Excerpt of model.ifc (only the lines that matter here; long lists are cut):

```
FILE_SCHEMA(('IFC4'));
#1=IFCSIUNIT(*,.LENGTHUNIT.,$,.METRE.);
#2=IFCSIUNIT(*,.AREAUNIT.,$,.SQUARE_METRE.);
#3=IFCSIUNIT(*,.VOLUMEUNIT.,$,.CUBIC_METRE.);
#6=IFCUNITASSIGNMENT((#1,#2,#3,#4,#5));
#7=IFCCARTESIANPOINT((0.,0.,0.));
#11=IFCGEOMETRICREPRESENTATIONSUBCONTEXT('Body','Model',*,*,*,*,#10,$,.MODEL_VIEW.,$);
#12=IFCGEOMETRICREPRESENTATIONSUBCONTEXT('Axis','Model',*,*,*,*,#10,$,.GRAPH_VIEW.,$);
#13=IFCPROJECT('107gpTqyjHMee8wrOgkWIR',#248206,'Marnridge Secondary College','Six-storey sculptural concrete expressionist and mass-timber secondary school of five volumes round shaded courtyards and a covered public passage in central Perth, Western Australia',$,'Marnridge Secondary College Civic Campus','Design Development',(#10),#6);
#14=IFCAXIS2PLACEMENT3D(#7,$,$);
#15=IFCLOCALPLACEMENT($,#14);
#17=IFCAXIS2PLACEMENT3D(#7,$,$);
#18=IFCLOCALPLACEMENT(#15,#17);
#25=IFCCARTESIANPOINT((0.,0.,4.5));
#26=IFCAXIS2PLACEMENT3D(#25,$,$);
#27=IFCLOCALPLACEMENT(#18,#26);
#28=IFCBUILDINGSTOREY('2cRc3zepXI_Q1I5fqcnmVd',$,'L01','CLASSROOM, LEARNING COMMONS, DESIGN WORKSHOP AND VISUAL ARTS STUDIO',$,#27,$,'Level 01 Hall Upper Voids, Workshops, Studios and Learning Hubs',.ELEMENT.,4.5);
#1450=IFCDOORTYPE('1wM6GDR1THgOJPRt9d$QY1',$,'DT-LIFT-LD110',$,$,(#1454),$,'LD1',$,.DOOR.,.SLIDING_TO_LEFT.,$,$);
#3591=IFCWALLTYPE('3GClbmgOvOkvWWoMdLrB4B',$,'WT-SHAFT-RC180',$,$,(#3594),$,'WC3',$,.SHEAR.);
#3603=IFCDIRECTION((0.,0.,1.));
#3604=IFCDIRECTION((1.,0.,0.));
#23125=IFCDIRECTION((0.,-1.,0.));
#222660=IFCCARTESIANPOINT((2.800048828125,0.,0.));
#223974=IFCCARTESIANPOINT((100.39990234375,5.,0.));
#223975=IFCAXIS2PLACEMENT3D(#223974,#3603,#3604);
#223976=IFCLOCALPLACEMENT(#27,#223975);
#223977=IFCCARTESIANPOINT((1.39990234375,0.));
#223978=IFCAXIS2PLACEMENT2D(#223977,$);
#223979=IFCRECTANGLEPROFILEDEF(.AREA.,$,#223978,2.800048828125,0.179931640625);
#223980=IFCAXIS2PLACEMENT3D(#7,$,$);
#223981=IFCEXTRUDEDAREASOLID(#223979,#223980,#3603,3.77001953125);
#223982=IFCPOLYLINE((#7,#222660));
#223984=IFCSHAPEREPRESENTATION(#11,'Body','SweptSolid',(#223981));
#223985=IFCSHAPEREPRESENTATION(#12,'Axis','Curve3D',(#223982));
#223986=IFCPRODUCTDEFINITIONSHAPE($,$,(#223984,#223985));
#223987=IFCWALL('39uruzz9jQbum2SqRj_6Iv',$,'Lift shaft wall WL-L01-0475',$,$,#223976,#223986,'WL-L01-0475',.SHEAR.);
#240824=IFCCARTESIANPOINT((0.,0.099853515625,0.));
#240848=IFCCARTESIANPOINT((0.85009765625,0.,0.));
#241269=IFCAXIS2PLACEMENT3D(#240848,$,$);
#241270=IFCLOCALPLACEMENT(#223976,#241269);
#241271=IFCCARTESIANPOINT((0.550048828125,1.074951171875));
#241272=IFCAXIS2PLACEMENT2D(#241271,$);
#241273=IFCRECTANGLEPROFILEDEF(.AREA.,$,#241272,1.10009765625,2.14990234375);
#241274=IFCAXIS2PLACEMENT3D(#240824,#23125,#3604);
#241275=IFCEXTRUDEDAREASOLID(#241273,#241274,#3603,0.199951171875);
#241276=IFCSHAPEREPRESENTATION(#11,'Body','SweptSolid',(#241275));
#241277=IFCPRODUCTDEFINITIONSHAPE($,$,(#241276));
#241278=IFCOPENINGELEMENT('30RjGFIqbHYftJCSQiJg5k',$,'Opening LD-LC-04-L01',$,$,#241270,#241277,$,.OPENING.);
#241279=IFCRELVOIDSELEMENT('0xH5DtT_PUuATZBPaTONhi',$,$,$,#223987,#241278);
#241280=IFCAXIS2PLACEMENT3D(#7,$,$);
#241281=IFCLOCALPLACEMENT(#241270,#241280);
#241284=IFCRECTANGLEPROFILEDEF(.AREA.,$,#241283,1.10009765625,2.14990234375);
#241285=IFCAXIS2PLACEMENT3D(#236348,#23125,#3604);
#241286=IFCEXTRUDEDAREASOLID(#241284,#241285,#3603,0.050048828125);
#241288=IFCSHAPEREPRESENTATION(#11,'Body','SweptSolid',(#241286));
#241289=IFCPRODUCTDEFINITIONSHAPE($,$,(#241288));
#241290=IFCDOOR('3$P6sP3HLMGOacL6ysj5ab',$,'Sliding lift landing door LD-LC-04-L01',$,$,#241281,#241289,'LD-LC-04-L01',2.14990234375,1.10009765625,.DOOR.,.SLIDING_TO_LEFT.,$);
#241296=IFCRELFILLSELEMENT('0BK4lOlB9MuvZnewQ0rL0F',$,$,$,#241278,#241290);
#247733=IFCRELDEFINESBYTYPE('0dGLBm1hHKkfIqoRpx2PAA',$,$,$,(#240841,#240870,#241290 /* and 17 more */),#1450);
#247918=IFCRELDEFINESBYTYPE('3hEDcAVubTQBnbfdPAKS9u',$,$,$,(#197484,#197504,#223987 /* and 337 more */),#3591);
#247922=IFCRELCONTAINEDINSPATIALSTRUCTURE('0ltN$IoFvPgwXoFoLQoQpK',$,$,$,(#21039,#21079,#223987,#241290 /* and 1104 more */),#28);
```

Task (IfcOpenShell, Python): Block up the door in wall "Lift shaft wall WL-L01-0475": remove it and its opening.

```python
import ifcopenshell
import ifcopenshell.api.feature
import ifcopenshell.api.root
import ifcopenshell.geom
import ifcopenshell.util.shape

model = ifcopenshell.open("model.ifc")
settings = ifcopenshell.geom.settings()


def volume(element):
    """Net volume in cubic metres, openings subtracted."""
    shape = ifcopenshell.geom.create_shape(settings, element)
    return ifcopenshell.util.shape.get_volume(shape.geometry)


door = model.by_guid("3$P6sP3HLMGOacL6ysj5ab")
opening = door.FillsVoids[0].RelatingOpeningElement
wall = opening.VoidsElements[0].RelatingBuildingElement
before = volume(wall)

ifcopenshell.api.root.remove_product(model, product=door)
ifcopenshell.api.feature.remove_feature(model, feature=opening)

after = volume(wall)

print(f"wall volume {before:.3f} -> {after:.3f} m3")

model.write("model_v2.ifc")
```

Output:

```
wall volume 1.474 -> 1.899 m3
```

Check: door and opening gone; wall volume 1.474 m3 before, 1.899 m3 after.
